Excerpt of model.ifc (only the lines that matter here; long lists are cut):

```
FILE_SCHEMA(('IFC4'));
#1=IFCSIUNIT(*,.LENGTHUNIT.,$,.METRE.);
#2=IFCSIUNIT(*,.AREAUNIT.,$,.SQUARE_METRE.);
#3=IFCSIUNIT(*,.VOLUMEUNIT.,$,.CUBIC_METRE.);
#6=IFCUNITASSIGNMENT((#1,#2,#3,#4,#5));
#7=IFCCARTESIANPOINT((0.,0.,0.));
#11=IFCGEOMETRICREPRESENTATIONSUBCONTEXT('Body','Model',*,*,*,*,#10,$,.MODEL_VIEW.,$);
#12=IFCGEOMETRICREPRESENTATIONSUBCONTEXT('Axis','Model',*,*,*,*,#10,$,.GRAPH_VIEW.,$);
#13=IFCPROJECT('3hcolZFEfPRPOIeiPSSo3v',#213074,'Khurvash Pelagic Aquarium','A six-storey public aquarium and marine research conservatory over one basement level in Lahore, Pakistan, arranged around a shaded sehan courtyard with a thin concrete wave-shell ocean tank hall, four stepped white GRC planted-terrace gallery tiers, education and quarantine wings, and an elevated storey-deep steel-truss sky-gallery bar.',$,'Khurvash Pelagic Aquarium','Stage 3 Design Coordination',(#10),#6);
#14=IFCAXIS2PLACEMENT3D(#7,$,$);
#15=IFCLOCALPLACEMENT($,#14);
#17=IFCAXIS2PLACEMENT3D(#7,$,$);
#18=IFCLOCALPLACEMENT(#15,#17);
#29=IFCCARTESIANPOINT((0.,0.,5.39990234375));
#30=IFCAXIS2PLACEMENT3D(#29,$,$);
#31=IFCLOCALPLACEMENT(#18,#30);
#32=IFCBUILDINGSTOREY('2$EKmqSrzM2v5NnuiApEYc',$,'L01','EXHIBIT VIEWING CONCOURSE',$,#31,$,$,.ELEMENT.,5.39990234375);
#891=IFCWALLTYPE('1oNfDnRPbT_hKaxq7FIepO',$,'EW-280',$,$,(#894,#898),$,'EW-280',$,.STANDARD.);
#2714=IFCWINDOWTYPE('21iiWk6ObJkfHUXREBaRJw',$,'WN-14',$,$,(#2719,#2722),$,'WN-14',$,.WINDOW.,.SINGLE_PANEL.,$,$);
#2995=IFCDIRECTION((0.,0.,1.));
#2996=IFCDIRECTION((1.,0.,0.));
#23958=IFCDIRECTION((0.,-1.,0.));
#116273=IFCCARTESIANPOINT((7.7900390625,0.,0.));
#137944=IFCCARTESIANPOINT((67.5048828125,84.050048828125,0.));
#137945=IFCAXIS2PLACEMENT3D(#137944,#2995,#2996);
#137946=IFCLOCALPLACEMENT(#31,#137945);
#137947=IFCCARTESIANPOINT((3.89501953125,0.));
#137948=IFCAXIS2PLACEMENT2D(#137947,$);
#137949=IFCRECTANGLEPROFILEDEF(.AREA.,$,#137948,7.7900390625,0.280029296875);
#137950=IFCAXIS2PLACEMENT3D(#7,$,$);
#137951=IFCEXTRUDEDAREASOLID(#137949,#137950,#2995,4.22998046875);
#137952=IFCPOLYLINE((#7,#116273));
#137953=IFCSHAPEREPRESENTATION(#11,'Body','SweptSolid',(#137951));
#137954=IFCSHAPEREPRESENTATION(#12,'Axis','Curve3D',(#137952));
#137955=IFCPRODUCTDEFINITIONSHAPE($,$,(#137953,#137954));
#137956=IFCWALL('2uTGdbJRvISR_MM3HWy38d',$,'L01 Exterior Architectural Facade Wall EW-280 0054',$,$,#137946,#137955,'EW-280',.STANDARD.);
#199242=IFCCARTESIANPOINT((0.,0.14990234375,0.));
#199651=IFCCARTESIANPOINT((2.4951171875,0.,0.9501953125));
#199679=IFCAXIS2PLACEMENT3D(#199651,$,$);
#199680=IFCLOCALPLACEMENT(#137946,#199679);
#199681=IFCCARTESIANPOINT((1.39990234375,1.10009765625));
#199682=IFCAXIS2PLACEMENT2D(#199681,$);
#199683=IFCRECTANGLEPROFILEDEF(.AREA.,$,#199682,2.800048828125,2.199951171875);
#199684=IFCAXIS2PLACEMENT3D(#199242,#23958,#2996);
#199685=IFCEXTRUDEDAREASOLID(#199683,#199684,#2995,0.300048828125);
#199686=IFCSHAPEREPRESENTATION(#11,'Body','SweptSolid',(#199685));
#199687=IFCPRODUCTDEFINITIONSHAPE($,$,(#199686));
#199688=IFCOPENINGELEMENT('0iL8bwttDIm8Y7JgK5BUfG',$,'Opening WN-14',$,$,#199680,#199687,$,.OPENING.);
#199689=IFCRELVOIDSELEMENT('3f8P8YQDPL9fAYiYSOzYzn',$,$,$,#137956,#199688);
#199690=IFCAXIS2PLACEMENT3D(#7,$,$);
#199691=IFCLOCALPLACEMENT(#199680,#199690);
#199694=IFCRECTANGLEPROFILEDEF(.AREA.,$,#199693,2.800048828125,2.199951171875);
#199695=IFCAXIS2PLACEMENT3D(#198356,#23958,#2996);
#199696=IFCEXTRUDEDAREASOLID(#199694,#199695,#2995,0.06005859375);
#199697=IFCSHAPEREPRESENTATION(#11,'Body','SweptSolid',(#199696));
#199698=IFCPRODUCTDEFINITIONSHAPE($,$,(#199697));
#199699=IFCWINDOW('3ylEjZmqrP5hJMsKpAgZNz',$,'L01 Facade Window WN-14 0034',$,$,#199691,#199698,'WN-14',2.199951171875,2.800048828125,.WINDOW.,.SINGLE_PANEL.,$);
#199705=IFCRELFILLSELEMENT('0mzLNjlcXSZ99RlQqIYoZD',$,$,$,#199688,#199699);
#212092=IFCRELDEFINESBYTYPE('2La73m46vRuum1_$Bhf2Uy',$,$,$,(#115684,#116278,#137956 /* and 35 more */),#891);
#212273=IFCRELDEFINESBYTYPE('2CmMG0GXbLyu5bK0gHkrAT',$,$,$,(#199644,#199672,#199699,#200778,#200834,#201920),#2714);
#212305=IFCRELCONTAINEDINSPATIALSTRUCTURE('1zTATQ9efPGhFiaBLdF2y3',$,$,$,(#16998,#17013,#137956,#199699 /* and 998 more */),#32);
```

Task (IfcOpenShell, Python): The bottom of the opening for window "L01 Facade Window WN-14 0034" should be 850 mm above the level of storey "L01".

```python
import numpy as np
import ifcopenshell
import ifcopenshell.api.geometry
import ifcopenshell.geom
import ifcopenshell.util.element
import ifcopenshell.util.placement
import ifcopenshell.util.shape
import ifcopenshell.util.unit

model = ifcopenshell.open("model.ifc")
unit_scale = ifcopenshell.util.unit.calculate_unit_scale(model)

window = model.by_guid("3ylEjZmqrP5hJMsKpAgZNz")
opening = window.FillsVoids[0].RelatingOpeningElement
storey = ifcopenshell.util.element.get_container(window, ifc_class="IfcBuildingStorey")
level = ifcopenshell.util.placement.get_local_placement(storey.ObjectPlacement)[2, 3]

# The opening's origin need not be at the sill, so measure its lowest point.
shape = ifcopenshell.geom.create_shape(ifcopenshell.geom.settings(), opening)
bottom = ifcopenshell.util.shape.get_shape_bottom_elevation(shape, shape.geometry) / unit_scale
dz = level + 0.85 - bottom

shift = np.array([0.0, 0.0, dz])
# The window is placed relative to its opening, so it follows when the opening moves.
matrix = ifcopenshell.util.placement.get_local_placement(opening.ObjectPlacement)
matrix[:3, 3] += shift
ifcopenshell.api.geometry.edit_object_placement(
    model, product=opening, matrix=matrix, is_si=False, should_transform_children=True
)

print(f"moved by {dz * unit_scale:+.3f} m")

model.write("model_updated.ifc")
```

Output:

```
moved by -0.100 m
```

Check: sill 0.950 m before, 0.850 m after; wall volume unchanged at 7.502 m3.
